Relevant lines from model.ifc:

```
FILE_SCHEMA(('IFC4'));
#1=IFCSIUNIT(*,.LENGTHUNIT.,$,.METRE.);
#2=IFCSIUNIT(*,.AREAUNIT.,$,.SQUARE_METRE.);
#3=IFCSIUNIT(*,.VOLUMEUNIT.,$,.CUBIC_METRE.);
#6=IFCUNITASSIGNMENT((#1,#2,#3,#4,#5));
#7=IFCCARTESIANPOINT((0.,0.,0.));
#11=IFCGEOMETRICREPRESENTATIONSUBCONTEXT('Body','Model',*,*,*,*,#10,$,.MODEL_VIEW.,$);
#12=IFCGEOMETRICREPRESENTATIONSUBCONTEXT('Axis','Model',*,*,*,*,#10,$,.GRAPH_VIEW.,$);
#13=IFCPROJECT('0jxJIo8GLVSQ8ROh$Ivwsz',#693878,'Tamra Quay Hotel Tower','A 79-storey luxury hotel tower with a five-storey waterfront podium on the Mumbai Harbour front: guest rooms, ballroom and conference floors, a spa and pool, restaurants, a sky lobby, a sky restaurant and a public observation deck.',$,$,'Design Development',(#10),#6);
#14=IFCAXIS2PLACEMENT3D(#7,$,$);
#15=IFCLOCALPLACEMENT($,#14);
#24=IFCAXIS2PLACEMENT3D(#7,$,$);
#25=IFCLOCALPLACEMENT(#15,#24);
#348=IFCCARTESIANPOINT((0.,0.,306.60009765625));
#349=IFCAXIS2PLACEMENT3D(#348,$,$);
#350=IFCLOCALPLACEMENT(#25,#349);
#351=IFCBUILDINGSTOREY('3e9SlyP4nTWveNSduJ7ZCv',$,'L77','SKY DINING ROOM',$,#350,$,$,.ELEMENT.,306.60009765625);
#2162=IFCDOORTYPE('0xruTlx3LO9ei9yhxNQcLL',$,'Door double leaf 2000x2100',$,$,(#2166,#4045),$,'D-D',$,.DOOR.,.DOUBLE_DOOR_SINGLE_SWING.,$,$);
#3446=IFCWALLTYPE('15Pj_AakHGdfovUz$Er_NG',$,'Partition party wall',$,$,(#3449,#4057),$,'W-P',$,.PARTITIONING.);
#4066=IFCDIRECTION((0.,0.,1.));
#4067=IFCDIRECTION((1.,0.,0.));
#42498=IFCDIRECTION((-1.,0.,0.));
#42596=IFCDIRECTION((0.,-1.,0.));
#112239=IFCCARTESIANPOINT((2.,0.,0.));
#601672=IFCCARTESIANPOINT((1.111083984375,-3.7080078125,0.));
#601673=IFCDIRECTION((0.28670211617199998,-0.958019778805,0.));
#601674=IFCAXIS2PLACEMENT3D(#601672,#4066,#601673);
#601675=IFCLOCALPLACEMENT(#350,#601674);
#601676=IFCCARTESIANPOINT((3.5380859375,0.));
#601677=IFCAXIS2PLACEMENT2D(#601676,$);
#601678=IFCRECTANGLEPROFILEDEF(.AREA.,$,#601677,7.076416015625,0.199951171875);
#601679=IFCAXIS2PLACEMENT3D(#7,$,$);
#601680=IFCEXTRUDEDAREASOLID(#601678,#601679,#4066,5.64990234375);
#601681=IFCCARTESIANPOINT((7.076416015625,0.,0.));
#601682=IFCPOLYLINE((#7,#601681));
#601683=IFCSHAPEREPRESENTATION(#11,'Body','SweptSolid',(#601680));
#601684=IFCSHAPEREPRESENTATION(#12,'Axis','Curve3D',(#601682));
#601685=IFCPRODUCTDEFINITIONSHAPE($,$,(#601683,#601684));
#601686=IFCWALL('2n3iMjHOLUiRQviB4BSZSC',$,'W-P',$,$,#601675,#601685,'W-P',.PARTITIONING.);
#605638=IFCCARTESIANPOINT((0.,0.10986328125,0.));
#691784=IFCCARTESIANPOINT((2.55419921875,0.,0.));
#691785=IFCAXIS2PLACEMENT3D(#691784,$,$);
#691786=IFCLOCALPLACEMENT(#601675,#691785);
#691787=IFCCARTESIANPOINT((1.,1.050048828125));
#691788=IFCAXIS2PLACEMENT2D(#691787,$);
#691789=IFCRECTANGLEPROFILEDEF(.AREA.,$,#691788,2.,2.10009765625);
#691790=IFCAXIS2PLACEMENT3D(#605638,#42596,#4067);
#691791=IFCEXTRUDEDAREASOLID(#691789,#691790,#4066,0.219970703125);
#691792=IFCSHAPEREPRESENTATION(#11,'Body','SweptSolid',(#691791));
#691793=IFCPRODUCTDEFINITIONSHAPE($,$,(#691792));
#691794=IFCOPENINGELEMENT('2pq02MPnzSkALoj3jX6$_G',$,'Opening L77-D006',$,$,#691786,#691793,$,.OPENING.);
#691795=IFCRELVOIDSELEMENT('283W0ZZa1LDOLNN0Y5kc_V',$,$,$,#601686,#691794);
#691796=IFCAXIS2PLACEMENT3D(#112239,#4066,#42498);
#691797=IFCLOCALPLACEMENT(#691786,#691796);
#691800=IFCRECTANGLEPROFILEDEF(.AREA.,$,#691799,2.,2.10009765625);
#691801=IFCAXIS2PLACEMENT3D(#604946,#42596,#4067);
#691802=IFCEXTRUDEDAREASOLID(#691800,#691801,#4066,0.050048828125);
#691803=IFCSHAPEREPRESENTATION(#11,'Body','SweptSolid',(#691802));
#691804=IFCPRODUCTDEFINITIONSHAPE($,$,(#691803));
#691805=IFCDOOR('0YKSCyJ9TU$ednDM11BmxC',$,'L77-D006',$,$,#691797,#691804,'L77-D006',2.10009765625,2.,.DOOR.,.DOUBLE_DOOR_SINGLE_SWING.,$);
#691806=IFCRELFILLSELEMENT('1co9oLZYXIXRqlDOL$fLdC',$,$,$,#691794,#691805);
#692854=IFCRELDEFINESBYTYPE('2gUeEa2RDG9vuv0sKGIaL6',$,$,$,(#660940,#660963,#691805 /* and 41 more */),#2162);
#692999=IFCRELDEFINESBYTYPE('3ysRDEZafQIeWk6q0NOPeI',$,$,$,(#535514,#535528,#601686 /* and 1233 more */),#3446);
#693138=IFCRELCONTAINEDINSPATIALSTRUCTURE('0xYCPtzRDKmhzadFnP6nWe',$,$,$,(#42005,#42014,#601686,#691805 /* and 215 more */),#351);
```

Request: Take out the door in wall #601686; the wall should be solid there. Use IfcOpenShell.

```python
import ifcopenshell
import ifcopenshell.api.feature
import ifcopenshell.api.root
import ifcopenshell.geom
import ifcopenshell.util.shape

model = ifcopenshell.open("model.ifc")
settings = ifcopenshell.geom.settings()


def volume(element):
    """Net volume in cubic metres, openings subtracted."""
    shape = ifcopenshell.geom.create_shape(settings, element)
    return ifcopenshell.util.shape.get_volume(shape.geometry)


door = model.by_guid("0YKSCyJ9TU$ednDM11BmxC")
opening = door.FillsVoids[0].RelatingOpeningElement
wall = opening.VoidsElements[0].RelatingBuildingElement
before = volume(wall)

ifcopenshell.api.root.remove_product(model, product=door)
ifcopenshell.api.feature.remove_feature(model, feature=opening)

after = volume(wall)

print(f"wall volume {before:.3f} -> {after:.3f} m3")

model.write("model_rev.ifc")
```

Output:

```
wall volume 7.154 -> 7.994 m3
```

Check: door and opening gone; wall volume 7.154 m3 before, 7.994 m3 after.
